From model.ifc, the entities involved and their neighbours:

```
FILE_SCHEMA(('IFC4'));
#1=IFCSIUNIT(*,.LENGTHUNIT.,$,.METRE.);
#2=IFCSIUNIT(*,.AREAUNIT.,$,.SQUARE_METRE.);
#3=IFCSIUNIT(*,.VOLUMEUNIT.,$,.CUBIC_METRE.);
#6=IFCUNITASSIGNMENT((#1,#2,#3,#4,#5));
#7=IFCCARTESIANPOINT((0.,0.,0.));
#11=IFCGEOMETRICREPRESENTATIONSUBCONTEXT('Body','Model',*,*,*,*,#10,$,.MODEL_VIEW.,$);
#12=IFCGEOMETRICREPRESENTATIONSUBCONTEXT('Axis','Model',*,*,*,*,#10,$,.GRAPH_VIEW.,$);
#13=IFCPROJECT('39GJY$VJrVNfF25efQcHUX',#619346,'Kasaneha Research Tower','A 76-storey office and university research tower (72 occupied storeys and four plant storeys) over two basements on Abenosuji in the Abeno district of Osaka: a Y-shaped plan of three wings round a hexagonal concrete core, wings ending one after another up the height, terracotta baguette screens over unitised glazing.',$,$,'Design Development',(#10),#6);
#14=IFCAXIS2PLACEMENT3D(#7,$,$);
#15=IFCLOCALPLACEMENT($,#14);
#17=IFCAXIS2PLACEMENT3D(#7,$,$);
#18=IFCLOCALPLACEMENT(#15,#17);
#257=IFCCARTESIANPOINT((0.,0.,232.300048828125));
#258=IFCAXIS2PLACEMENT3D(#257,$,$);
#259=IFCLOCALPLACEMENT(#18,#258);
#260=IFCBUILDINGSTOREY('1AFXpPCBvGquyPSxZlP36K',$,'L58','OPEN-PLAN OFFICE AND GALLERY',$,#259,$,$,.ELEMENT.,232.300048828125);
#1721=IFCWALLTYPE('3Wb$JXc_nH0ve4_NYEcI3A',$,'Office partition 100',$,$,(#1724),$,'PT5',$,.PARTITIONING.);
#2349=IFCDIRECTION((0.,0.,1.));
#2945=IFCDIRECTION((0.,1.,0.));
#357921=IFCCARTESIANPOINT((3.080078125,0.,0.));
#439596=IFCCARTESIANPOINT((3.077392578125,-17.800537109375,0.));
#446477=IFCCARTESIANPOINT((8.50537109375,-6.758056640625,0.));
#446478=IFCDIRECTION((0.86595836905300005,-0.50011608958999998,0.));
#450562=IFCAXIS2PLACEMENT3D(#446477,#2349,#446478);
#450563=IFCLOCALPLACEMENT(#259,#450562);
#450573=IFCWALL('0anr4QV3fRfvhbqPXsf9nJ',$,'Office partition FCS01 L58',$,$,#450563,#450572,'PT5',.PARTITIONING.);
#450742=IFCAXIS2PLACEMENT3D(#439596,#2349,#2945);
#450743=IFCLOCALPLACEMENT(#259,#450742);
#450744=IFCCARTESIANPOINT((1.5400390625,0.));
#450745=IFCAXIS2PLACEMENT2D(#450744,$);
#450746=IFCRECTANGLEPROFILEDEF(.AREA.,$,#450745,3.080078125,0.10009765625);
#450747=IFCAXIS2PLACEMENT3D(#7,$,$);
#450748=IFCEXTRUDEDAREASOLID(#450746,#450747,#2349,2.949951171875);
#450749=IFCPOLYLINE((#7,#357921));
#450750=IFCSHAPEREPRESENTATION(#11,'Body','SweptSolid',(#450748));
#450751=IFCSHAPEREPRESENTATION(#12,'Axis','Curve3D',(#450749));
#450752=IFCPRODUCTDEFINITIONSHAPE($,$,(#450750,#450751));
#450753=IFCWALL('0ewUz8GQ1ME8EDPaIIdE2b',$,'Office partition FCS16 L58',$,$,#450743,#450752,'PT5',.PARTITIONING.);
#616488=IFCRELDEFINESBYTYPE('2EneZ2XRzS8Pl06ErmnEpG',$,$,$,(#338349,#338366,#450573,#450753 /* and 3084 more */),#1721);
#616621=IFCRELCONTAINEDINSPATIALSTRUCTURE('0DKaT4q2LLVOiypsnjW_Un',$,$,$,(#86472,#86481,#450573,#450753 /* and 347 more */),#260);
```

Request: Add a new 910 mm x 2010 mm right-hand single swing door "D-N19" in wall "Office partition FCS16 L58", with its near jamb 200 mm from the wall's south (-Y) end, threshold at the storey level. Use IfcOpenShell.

```python
import numpy as np
import ifcopenshell
import ifcopenshell.api.feature
import ifcopenshell.api.geometry
import ifcopenshell.api.root
import ifcopenshell.api.spatial
import ifcopenshell.geom
import ifcopenshell.util.element
import ifcopenshell.util.placement
import ifcopenshell.util.representation
import ifcopenshell.util.shape
import ifcopenshell.util.unit

model = ifcopenshell.open("model.ifc")
unit_scale = ifcopenshell.util.unit.calculate_unit_scale(model)
settings = ifcopenshell.geom.settings()


def volume(element):
    """Net volume in cubic metres, openings subtracted."""
    shape = ifcopenshell.geom.create_shape(settings, element)
    return ifcopenshell.util.shape.get_volume(shape.geometry)


wall = model.by_guid("0ewUz8GQ1ME8EDPaIIdE2b")
storey = ifcopenshell.util.element.get_container(wall, ifc_class="IfcBuildingStorey")
context = ifcopenshell.util.representation.get_context(model, "Model", "Body", "MODEL_VIEW")
before = volume(wall)

width, height, from_end, sill = 0.91, 2.01, 0.2, 0.0  # metres

# The wall runs along its own X axis, and the end named is its -X end.
wall_shape = ifcopenshell.geom.create_shape(settings, wall)
x, y, z = ifcopenshell.util.shape.get_vertices(wall_shape.geometry).T
start = x.min() + from_end
face, thickness = float(y.min()), float(y.max() - y.min())
wall_matrix = ifcopenshell.util.placement.get_local_placement(wall.ObjectPlacement)
level = ifcopenshell.util.placement.get_local_placement(storey.ObjectPlacement)[2, 3]


def in_wall(x, y):
    """Placement at x, y metres in the wall's axes, at sill height."""
    matrix = wall_matrix.copy()
    matrix[:, 3] = wall_matrix @ np.array([x / unit_scale, y / unit_scale, 0.0, 1.0])
    matrix[2, 3] = level + sill / unit_scale
    return matrix


# Opening: a box that overshoots both wall faces by 50 mm.
opening = ifcopenshell.api.root.create_entity(model, ifc_class="IfcOpeningElement", predefined_type="OPENING")
box = ifcopenshell.api.geometry.add_wall_representation(
    model, context=context, length=width, height=height, thickness=thickness + 0.1
)
ifcopenshell.api.geometry.assign_representation(model, product=opening, representation=box)
ifcopenshell.api.geometry.edit_object_placement(model, product=opening, matrix=in_wall(start, face - 0.05), is_si=False)
ifcopenshell.api.feature.add_feature(model, feature=opening, element=wall)

door = ifcopenshell.api.root.create_entity(model, ifc_class="IfcDoor", name="D-N19", predefined_type="DOOR")
door.OverallWidth, door.OverallHeight = width / unit_scale, height / unit_scale
door.OperationType = "SINGLE_SWING_RIGHT"
body = ifcopenshell.api.geometry.add_door_representation(
    model,
    context=context,
    overall_width=door.OverallWidth,
    overall_height=door.OverallHeight,
    operation_type="SINGLE_SWING_RIGHT",
    lining_properties={"LiningDepth": thickness / unit_scale, "ThresholdDepth": thickness / unit_scale},
)
ifcopenshell.api.geometry.assign_representation(model, product=door, representation=body)
ifcopenshell.api.spatial.assign_container(model, products=[door], relating_structure=storey)
ifcopenshell.api.feature.add_filling(model, opening=opening, element=door)

# The lining spans the wall, so the door starts at the wall face.
ifcopenshell.api.geometry.edit_object_placement(model, product=door, matrix=in_wall(start, face), is_si=False)

after = volume(wall)

print(f"wall volume {before:.3f} -> {after:.3f} m3")

model.write("model-out.ifc")
```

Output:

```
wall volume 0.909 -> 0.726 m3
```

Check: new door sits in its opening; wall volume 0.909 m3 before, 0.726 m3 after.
